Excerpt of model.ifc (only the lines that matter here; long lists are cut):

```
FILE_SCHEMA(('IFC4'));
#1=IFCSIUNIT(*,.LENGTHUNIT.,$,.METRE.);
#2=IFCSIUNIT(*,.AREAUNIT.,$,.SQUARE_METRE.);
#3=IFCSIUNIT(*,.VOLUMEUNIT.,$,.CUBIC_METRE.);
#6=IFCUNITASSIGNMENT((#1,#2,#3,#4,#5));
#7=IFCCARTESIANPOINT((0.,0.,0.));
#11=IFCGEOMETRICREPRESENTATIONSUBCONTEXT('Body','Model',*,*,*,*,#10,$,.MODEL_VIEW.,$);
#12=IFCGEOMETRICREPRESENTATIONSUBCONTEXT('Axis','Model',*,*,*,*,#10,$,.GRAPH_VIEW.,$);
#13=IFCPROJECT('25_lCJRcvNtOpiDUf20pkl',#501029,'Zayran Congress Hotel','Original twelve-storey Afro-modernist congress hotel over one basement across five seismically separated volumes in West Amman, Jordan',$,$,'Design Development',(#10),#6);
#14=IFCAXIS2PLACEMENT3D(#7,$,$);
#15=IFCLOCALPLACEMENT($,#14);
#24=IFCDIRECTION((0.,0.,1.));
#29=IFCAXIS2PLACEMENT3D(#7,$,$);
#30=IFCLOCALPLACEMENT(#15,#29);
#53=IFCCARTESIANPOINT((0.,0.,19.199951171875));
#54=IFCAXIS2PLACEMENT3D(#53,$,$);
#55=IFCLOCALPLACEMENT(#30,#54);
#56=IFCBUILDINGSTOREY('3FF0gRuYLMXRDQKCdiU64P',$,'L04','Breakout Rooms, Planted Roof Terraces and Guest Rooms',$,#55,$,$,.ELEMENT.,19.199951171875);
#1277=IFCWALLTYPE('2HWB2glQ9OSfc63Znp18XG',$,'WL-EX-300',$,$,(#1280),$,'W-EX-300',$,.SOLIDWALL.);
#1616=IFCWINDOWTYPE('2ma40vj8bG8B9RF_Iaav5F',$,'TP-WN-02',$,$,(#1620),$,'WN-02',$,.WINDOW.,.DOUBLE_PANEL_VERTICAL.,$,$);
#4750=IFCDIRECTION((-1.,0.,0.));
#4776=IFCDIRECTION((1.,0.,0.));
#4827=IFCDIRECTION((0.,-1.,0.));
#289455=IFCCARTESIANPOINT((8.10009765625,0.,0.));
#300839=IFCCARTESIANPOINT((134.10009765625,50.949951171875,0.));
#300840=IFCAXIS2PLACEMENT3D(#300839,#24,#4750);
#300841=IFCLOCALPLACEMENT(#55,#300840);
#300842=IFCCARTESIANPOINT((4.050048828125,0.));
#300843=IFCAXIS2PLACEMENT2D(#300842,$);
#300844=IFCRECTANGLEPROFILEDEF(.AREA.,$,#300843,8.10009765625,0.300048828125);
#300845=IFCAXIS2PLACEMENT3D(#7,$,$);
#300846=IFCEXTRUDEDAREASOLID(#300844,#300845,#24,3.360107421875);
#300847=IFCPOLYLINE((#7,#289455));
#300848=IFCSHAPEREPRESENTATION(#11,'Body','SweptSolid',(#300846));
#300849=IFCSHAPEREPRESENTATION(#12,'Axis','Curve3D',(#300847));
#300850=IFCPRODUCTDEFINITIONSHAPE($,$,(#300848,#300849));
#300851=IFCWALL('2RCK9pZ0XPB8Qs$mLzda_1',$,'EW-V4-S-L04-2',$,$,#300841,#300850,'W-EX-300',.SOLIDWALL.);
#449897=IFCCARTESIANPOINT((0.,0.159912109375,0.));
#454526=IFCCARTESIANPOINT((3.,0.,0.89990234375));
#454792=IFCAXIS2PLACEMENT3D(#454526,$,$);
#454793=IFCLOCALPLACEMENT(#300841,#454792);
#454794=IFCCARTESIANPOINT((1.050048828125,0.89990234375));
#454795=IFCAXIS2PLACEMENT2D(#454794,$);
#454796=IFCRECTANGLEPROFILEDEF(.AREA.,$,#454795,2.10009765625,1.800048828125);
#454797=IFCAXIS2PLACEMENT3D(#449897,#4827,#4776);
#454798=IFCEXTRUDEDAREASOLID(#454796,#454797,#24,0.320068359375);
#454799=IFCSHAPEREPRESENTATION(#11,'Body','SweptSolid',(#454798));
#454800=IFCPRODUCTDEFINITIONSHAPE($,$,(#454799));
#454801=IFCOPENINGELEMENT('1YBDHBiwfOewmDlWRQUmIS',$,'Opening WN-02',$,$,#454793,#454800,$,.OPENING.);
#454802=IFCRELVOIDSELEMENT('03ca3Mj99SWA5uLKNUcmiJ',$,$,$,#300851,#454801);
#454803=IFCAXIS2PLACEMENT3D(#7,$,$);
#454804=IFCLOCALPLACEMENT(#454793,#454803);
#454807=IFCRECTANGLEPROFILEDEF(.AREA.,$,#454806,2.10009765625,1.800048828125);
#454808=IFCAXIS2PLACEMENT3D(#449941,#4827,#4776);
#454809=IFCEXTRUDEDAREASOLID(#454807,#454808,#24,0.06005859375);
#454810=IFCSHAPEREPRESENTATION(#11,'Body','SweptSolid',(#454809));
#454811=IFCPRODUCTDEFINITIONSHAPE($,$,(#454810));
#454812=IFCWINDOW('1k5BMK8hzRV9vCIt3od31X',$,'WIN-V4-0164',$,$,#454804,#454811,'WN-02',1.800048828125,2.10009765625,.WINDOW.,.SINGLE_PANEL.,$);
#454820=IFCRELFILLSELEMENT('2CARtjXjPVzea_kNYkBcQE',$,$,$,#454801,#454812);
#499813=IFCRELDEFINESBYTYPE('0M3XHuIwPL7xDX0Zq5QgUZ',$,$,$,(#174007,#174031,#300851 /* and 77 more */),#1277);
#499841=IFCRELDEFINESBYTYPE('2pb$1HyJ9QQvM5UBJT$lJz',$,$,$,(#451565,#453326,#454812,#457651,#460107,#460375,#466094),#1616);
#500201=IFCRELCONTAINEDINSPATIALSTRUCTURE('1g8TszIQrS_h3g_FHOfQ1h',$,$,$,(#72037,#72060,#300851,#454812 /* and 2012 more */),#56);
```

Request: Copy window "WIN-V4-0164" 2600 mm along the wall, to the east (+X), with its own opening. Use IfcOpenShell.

```python
import ifcopenshell
import ifcopenshell.api.feature
import ifcopenshell.api.geometry
import ifcopenshell.api.root
import ifcopenshell.geom
import ifcopenshell.util.element
import ifcopenshell.util.placement
import ifcopenshell.util.shape
import ifcopenshell.util.unit

model = ifcopenshell.open("model.ifc")
unit_scale = ifcopenshell.util.unit.calculate_unit_scale(model)
settings = ifcopenshell.geom.settings()


def volume(element):
    """Net volume in cubic metres, openings subtracted."""
    shape = ifcopenshell.geom.create_shape(settings, element)
    return ifcopenshell.util.shape.get_volume(shape.geometry)


window = model.by_guid("1k5BMK8hzRV9vCIt3od31X")
opening = window.FillsVoids[0].RelatingOpeningElement
wall = opening.VoidsElements[0].RelatingBuildingElement
before = volume(wall)
shift = ifcopenshell.util.placement.get_local_placement(wall.ObjectPlacement)[:3, 0] * -2.6 / unit_scale

# copy_class copies the void relationship, type, container and properties, but no geometry.
new_opening = ifcopenshell.api.root.copy_class(model, product=opening)
new_opening.Representation = ifcopenshell.util.element.copy_deep(
    model, opening.Representation, exclude=["IfcGeometricRepresentationContext", "IfcRepresentationMap"]
)
new_window = ifcopenshell.api.root.copy_class(model, product=window)
new_window.Representation = ifcopenshell.util.element.copy_deep(
    model, window.Representation, exclude=["IfcGeometricRepresentationContext", "IfcRepresentationMap"]
)
new_window.Tag = None
ifcopenshell.api.feature.add_filling(model, opening=new_opening, element=new_window)

for old, new in ((opening, new_opening), (window, new_window)):
    matrix = ifcopenshell.util.placement.get_local_placement(old.ObjectPlacement)
    matrix[:3, 3] += shift
    ifcopenshell.api.geometry.edit_object_placement(model, product=new, matrix=matrix, is_si=False)

after = volume(wall)

print(f"wall volume {before:.3f} -> {after:.3f} m3")

model.write("model_v2.ifc")
```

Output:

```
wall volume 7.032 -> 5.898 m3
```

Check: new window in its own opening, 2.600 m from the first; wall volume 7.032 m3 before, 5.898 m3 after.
